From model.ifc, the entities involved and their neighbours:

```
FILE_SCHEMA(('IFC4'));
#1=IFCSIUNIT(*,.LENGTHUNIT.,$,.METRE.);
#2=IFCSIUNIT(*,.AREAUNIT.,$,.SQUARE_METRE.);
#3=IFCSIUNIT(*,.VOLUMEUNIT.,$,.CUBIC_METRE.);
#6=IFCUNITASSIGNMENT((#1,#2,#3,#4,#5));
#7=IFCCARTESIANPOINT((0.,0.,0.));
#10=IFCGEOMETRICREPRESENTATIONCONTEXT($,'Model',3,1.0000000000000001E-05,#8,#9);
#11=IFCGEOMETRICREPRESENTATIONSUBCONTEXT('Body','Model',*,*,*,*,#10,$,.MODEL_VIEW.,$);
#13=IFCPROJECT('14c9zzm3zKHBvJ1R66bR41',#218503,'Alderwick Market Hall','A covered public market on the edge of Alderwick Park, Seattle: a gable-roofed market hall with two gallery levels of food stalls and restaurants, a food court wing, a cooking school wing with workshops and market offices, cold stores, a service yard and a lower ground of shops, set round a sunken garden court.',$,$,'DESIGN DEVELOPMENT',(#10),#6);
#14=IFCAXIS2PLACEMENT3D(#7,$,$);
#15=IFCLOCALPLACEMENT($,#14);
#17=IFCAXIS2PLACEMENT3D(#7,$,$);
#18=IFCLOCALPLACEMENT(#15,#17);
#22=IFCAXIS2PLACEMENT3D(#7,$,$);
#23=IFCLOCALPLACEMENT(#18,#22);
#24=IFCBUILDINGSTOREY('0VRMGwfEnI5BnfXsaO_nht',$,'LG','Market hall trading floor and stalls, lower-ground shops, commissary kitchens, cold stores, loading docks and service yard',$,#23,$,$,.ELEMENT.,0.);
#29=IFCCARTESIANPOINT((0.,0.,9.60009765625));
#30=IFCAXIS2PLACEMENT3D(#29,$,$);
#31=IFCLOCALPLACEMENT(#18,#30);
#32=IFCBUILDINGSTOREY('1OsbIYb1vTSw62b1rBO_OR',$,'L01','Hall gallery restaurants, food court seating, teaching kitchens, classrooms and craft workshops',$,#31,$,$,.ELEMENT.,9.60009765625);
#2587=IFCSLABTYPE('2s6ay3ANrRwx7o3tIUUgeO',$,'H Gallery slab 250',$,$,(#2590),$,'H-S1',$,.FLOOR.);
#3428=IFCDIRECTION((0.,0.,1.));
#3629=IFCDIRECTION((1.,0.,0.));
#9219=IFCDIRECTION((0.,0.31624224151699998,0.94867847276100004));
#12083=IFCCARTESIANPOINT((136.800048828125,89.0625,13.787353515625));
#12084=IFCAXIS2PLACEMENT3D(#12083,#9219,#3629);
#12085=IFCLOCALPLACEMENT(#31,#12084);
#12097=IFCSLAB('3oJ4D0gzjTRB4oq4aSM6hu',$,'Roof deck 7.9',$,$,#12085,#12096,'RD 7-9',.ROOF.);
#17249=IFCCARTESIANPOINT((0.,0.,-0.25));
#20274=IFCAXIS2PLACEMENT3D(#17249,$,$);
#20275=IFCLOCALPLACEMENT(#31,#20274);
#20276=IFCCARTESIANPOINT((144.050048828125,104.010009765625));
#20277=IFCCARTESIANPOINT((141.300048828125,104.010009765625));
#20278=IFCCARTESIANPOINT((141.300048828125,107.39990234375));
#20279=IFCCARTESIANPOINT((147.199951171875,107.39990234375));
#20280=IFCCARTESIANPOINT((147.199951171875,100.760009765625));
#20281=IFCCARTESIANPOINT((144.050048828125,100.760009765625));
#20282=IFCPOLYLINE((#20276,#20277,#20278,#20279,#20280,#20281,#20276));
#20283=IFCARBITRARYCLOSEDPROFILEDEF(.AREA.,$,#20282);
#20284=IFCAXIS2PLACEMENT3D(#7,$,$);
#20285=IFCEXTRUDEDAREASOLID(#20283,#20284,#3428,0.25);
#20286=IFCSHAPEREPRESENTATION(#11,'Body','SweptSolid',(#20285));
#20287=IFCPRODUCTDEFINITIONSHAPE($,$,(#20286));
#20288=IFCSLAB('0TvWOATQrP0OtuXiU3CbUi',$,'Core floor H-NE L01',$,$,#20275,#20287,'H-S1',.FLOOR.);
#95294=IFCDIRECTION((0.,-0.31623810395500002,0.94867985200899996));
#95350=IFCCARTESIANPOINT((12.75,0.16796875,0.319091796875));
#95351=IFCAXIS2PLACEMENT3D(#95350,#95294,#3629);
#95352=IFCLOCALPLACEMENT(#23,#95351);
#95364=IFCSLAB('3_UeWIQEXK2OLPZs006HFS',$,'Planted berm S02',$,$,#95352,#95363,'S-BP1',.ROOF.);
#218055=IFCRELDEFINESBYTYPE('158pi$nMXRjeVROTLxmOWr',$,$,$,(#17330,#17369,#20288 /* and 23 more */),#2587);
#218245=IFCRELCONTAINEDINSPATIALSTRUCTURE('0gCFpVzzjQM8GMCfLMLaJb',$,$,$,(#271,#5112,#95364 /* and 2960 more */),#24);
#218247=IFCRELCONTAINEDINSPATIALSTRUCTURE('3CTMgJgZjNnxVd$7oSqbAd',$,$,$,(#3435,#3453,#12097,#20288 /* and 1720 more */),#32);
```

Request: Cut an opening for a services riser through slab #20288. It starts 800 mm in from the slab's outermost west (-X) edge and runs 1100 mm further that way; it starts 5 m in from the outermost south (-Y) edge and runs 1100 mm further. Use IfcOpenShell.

```python
import numpy as np
import ifcopenshell
import ifcopenshell.api.feature
import ifcopenshell.api.geometry
import ifcopenshell.api.root
import ifcopenshell.geom
import ifcopenshell.util.placement
import ifcopenshell.util.representation
import ifcopenshell.util.shape
import ifcopenshell.util.unit

model = ifcopenshell.open("model.ifc")
unit_scale = ifcopenshell.util.unit.calculate_unit_scale(model)
settings = ifcopenshell.geom.settings()


def volume(element):
    """Net volume in cubic metres, openings subtracted."""
    shape = ifcopenshell.geom.create_shape(settings, element)
    return ifcopenshell.util.shape.get_volume(shape.geometry)


slab = model.by_guid("0TvWOATQrP0OtuXiU3CbUi")
before = volume(slab)

# Extent in the slab's own axes, in metres. The edges named are its -X and -Y sides.
slab_shape = ifcopenshell.geom.create_shape(settings, slab)
vertices = ifcopenshell.util.shape.get_vertices(slab_shape.geometry)
x_min, y_min, bottom = vertices.min(axis=0)
top = vertices[:, 2].max()

opening = ifcopenshell.api.root.create_entity(model, ifc_class="IfcOpeningElement", name="Services riser opening", predefined_type="OPENING")
context = ifcopenshell.util.representation.get_context(model, "Model", "Body", "MODEL_VIEW")
width, depth = 1.1, 1.1
outline = [(0.0, 0.0), (width, 0.0), (width, depth), (0.0, depth), (0.0, 0.0)]
# Overshoot both faces by 50 mm so the cut is clean.
shape = ifcopenshell.api.geometry.add_slab_representation(
    model, context=context, depth=top - bottom + 0.1, polyline=outline
)
ifcopenshell.api.geometry.assign_representation(model, product=opening, representation=shape)

matrix = ifcopenshell.util.placement.get_local_placement(slab.ObjectPlacement)
matrix[:, 3] = matrix @ np.append(np.array([x_min + 0.8, y_min + 5, bottom - 0.05]) / unit_scale, 1.0)
ifcopenshell.api.geometry.edit_object_placement(model, product=opening, matrix=matrix, is_si=False)
ifcopenshell.api.feature.add_feature(model, feature=opening, element=slab)

after = volume(slab)

print(f"slab volume {before:.3f} -> {after:.3f} m3")

model.write("model_edited.ifc")
```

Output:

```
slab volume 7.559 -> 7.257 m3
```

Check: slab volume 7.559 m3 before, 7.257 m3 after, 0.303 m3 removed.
